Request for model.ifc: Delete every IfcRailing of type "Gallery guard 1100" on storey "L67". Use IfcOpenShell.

First a look at what the model holds.

```python
import ifcopenshell
import ifcopenshell.util.element

model = ifcopenshell.open("model.ifc")
print(model.schema)
storey = next(s for s in model.by_type("IfcBuildingStorey") if s.Name == "L67")
railings = [e for e in ifcopenshell.util.element.get_decomposition(storey) if e.is_a("IfcRailing")]
seen = {}
for e in railings:
    element_type = ifcopenshell.util.element.get_type(e)
    name = element_type.Name if element_type not in (None, e) else None
    seen[name] = seen.get(name, 0) + 1
for name, count in sorted(seen.items(), key=str):
    print(count, "x", name)
```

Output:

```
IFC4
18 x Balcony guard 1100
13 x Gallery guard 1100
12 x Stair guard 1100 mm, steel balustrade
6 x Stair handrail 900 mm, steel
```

```python
import ifcopenshell
import ifcopenshell.api.root
import ifcopenshell.util.element

model = ifcopenshell.open("model.ifc")

storey = next(s for s in model.by_type("IfcBuildingStorey") if s.Name == "L67")
railings = [e for e in ifcopenshell.util.element.get_decomposition(storey) if e.is_a("IfcRailing")]
targets = [e for e in railings if (t := ifcopenshell.util.element.get_type(e)) not in (None, e) and t.Name == "Gallery guard 1100"]

for e in targets:
    ifcopenshell.api.root.remove_product(model, product=e)
print(len(targets), "removed")

model.write("model_v2.ifc")
```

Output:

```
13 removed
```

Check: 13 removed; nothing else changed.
